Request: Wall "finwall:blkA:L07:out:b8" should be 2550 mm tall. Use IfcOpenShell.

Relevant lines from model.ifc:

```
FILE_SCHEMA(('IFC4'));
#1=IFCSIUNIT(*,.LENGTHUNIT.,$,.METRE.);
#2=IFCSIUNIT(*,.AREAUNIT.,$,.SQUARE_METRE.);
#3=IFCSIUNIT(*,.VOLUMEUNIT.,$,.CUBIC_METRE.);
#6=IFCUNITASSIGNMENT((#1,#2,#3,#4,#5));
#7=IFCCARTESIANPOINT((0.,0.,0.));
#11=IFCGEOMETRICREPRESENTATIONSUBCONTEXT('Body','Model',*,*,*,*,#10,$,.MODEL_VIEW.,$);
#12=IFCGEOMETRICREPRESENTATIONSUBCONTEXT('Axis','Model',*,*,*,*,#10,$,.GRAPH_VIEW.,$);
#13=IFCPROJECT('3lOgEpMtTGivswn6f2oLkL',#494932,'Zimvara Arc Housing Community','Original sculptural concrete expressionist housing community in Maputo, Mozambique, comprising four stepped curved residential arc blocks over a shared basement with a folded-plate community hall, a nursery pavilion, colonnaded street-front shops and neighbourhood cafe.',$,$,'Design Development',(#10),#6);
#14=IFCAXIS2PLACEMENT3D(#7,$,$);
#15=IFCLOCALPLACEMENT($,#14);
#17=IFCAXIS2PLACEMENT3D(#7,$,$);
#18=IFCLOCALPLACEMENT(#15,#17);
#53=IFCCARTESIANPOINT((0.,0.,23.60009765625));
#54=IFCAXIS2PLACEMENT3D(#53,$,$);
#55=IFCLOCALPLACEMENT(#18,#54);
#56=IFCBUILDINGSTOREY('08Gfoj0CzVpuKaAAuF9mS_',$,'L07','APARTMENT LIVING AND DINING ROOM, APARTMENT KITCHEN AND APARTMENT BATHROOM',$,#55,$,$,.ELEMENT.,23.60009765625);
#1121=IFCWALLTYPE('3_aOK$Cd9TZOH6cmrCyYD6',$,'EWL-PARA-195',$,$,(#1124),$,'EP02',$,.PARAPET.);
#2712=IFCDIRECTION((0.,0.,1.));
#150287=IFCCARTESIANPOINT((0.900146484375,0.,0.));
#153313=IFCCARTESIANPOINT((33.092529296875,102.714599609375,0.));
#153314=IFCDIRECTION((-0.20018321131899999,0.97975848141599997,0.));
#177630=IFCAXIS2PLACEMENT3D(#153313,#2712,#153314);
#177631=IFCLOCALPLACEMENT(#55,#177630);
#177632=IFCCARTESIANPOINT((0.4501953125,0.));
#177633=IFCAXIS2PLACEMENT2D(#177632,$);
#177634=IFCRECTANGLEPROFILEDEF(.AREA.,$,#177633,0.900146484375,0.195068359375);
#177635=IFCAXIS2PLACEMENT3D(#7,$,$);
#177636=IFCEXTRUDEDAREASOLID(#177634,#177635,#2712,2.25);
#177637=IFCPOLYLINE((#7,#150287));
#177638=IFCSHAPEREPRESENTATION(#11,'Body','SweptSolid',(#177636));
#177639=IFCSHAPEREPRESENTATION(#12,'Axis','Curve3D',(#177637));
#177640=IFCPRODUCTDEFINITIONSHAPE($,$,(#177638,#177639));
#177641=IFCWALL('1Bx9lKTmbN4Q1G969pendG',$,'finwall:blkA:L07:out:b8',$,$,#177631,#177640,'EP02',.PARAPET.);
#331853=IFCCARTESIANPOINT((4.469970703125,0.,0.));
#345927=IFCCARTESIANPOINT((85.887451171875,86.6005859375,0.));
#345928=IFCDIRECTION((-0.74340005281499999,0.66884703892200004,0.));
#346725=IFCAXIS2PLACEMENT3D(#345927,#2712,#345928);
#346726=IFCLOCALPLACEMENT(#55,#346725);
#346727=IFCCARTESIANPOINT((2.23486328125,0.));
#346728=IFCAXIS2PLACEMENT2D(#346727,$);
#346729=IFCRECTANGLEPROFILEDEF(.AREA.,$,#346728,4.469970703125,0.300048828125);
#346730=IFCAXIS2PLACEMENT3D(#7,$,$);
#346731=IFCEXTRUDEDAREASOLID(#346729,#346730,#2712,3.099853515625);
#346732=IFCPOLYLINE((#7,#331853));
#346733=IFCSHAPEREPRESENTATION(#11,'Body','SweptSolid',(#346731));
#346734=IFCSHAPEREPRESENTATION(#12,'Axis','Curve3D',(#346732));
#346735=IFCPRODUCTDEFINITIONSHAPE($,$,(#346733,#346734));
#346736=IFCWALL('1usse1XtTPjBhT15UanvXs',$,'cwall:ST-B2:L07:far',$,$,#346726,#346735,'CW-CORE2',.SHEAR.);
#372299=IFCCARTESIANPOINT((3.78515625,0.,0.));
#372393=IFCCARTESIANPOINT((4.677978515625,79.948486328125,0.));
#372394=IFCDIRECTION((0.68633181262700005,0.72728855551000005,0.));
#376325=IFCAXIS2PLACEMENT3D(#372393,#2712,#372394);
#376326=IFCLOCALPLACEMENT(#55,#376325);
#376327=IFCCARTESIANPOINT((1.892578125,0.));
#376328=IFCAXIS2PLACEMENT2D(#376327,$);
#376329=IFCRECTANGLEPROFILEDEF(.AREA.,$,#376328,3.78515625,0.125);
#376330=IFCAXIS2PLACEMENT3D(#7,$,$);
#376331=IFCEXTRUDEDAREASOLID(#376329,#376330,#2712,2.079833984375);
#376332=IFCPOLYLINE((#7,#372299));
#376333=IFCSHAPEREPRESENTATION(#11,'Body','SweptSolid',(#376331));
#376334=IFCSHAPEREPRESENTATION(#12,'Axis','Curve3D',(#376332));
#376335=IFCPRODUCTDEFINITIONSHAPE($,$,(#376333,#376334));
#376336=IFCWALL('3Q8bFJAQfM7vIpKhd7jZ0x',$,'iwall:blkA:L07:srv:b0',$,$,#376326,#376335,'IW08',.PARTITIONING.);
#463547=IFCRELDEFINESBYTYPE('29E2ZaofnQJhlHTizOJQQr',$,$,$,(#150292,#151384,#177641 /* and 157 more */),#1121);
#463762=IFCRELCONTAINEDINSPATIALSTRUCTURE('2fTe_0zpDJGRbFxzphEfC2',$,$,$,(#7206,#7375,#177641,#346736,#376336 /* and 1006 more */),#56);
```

```python
import ifcopenshell
import ifcopenshell.geom
import ifcopenshell.util.representation
import ifcopenshell.util.shape

model = ifcopenshell.open("model.ifc")
settings = ifcopenshell.geom.settings()


def volume(element):
    """Net volume in cubic metres, openings subtracted."""
    shape = ifcopenshell.geom.create_shape(settings, element)
    return ifcopenshell.util.shape.get_volume(shape.geometry)


wall = model.by_guid("1Bx9lKTmbN4Q1G969pendG")
before = volume(wall)

body = ifcopenshell.util.representation.get_representation(wall, "Model", "Body")
solid = body.Items[0]
old_height = solid.Depth
solid.Depth = 2.55
after = volume(wall)

print(f"height {old_height:g} -> {solid.Depth:g}, volume {before:.3f} -> {after:.3f} m3")

model.write("model_v2.ifc")
```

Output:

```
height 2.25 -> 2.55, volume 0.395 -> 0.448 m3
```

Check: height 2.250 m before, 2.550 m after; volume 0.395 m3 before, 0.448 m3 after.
